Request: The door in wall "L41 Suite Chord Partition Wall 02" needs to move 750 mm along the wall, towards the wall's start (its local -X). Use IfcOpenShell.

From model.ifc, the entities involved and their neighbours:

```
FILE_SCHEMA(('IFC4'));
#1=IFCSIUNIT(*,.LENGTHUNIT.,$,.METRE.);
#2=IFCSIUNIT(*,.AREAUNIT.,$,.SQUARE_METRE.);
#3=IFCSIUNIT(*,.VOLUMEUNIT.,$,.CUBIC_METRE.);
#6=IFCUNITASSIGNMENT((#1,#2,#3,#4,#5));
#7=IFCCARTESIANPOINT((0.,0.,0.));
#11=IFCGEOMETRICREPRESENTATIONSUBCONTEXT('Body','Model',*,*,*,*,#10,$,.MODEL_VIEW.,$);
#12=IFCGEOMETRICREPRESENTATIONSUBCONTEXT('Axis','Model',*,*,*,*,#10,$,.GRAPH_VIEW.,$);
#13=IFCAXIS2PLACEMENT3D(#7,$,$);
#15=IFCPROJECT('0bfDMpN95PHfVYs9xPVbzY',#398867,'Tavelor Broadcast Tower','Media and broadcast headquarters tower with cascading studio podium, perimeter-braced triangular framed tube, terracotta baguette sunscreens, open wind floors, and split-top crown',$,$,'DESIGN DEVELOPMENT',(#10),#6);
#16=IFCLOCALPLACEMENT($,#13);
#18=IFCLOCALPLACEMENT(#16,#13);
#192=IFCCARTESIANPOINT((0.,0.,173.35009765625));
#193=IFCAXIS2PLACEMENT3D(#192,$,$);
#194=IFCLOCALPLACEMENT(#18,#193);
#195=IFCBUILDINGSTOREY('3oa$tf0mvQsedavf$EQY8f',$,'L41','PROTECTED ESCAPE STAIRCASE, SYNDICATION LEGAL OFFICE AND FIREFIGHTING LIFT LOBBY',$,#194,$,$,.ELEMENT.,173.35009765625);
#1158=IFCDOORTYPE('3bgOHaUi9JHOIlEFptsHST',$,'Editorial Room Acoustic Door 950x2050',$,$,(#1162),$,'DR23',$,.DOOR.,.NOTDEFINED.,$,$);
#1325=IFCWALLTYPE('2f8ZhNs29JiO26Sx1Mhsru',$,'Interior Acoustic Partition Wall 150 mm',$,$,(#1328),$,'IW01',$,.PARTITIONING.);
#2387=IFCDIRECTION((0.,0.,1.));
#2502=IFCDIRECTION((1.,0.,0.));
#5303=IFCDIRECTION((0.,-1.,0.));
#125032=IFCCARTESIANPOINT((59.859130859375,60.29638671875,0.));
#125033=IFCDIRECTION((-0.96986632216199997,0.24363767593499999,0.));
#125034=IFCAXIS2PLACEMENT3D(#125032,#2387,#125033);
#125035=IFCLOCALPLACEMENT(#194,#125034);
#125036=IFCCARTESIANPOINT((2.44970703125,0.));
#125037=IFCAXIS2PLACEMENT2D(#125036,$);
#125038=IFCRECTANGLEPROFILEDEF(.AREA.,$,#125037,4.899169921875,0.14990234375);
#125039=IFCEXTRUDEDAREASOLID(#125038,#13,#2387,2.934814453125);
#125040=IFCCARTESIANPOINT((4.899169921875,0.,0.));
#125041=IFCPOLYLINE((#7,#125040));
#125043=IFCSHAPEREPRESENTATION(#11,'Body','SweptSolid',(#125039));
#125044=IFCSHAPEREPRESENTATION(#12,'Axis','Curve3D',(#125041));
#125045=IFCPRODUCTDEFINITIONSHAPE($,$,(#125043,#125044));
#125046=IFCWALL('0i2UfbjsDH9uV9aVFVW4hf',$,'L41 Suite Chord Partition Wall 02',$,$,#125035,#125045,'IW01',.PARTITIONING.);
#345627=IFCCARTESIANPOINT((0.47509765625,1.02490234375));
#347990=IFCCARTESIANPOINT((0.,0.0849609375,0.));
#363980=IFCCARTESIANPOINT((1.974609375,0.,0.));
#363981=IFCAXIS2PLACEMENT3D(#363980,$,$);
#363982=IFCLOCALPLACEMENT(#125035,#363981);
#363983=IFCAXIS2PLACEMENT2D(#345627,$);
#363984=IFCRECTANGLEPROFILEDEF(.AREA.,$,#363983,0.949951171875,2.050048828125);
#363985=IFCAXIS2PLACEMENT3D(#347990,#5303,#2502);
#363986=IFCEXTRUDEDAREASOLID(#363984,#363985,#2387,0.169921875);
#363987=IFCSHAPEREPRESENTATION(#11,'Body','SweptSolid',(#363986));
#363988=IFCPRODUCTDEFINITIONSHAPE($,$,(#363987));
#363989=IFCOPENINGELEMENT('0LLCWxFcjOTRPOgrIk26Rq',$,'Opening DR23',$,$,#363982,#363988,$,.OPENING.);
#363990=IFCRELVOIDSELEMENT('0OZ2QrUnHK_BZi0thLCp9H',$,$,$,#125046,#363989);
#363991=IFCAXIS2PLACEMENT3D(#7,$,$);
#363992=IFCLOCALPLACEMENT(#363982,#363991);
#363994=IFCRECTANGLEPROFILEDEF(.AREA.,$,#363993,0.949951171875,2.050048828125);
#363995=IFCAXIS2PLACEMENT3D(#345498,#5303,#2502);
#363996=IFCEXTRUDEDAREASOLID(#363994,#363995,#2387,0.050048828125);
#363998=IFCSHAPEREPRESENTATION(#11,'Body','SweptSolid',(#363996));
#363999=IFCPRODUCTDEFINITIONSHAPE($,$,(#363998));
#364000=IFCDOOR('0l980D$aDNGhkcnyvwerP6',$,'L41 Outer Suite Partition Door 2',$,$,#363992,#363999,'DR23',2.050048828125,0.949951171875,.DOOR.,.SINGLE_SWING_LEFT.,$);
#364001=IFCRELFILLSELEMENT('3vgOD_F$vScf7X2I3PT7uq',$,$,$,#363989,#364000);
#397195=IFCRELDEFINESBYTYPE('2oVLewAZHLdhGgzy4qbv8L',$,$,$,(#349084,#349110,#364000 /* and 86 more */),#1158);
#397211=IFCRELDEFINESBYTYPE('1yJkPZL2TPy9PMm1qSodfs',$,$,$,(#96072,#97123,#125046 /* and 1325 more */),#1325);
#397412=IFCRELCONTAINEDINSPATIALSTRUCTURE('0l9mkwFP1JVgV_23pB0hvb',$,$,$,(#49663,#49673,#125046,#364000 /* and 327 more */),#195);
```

```python
import ifcopenshell
import ifcopenshell.api.geometry
import ifcopenshell.util.placement

model = ifcopenshell.open("model.ifc")

door = model.by_guid("0l980D$aDNGhkcnyvwerP6")
opening = door.FillsVoids[0].RelatingOpeningElement
wall = opening.VoidsElements[0].RelatingBuildingElement

wall_matrix = ifcopenshell.util.placement.get_local_placement(wall.ObjectPlacement)
shift = wall_matrix[:3, 0] * -0.75
before = ifcopenshell.util.placement.get_local_placement(door.ObjectPlacement)[:3, 3].copy()

# The door is placed relative to its opening, so it follows when the opening moves.
matrix = ifcopenshell.util.placement.get_local_placement(opening.ObjectPlacement)
matrix[:3, 3] += shift
ifcopenshell.api.geometry.edit_object_placement(
    model, product=opening, matrix=matrix, is_si=False, should_transform_children=True
)

after = ifcopenshell.util.placement.get_local_placement(door.ObjectPlacement)[:3, 3]
print("door moved by", (after - before).round(3) + 0.0)

model.write("model-out.ifc")
```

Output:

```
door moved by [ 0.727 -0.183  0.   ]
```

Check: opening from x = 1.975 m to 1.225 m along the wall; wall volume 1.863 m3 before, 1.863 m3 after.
